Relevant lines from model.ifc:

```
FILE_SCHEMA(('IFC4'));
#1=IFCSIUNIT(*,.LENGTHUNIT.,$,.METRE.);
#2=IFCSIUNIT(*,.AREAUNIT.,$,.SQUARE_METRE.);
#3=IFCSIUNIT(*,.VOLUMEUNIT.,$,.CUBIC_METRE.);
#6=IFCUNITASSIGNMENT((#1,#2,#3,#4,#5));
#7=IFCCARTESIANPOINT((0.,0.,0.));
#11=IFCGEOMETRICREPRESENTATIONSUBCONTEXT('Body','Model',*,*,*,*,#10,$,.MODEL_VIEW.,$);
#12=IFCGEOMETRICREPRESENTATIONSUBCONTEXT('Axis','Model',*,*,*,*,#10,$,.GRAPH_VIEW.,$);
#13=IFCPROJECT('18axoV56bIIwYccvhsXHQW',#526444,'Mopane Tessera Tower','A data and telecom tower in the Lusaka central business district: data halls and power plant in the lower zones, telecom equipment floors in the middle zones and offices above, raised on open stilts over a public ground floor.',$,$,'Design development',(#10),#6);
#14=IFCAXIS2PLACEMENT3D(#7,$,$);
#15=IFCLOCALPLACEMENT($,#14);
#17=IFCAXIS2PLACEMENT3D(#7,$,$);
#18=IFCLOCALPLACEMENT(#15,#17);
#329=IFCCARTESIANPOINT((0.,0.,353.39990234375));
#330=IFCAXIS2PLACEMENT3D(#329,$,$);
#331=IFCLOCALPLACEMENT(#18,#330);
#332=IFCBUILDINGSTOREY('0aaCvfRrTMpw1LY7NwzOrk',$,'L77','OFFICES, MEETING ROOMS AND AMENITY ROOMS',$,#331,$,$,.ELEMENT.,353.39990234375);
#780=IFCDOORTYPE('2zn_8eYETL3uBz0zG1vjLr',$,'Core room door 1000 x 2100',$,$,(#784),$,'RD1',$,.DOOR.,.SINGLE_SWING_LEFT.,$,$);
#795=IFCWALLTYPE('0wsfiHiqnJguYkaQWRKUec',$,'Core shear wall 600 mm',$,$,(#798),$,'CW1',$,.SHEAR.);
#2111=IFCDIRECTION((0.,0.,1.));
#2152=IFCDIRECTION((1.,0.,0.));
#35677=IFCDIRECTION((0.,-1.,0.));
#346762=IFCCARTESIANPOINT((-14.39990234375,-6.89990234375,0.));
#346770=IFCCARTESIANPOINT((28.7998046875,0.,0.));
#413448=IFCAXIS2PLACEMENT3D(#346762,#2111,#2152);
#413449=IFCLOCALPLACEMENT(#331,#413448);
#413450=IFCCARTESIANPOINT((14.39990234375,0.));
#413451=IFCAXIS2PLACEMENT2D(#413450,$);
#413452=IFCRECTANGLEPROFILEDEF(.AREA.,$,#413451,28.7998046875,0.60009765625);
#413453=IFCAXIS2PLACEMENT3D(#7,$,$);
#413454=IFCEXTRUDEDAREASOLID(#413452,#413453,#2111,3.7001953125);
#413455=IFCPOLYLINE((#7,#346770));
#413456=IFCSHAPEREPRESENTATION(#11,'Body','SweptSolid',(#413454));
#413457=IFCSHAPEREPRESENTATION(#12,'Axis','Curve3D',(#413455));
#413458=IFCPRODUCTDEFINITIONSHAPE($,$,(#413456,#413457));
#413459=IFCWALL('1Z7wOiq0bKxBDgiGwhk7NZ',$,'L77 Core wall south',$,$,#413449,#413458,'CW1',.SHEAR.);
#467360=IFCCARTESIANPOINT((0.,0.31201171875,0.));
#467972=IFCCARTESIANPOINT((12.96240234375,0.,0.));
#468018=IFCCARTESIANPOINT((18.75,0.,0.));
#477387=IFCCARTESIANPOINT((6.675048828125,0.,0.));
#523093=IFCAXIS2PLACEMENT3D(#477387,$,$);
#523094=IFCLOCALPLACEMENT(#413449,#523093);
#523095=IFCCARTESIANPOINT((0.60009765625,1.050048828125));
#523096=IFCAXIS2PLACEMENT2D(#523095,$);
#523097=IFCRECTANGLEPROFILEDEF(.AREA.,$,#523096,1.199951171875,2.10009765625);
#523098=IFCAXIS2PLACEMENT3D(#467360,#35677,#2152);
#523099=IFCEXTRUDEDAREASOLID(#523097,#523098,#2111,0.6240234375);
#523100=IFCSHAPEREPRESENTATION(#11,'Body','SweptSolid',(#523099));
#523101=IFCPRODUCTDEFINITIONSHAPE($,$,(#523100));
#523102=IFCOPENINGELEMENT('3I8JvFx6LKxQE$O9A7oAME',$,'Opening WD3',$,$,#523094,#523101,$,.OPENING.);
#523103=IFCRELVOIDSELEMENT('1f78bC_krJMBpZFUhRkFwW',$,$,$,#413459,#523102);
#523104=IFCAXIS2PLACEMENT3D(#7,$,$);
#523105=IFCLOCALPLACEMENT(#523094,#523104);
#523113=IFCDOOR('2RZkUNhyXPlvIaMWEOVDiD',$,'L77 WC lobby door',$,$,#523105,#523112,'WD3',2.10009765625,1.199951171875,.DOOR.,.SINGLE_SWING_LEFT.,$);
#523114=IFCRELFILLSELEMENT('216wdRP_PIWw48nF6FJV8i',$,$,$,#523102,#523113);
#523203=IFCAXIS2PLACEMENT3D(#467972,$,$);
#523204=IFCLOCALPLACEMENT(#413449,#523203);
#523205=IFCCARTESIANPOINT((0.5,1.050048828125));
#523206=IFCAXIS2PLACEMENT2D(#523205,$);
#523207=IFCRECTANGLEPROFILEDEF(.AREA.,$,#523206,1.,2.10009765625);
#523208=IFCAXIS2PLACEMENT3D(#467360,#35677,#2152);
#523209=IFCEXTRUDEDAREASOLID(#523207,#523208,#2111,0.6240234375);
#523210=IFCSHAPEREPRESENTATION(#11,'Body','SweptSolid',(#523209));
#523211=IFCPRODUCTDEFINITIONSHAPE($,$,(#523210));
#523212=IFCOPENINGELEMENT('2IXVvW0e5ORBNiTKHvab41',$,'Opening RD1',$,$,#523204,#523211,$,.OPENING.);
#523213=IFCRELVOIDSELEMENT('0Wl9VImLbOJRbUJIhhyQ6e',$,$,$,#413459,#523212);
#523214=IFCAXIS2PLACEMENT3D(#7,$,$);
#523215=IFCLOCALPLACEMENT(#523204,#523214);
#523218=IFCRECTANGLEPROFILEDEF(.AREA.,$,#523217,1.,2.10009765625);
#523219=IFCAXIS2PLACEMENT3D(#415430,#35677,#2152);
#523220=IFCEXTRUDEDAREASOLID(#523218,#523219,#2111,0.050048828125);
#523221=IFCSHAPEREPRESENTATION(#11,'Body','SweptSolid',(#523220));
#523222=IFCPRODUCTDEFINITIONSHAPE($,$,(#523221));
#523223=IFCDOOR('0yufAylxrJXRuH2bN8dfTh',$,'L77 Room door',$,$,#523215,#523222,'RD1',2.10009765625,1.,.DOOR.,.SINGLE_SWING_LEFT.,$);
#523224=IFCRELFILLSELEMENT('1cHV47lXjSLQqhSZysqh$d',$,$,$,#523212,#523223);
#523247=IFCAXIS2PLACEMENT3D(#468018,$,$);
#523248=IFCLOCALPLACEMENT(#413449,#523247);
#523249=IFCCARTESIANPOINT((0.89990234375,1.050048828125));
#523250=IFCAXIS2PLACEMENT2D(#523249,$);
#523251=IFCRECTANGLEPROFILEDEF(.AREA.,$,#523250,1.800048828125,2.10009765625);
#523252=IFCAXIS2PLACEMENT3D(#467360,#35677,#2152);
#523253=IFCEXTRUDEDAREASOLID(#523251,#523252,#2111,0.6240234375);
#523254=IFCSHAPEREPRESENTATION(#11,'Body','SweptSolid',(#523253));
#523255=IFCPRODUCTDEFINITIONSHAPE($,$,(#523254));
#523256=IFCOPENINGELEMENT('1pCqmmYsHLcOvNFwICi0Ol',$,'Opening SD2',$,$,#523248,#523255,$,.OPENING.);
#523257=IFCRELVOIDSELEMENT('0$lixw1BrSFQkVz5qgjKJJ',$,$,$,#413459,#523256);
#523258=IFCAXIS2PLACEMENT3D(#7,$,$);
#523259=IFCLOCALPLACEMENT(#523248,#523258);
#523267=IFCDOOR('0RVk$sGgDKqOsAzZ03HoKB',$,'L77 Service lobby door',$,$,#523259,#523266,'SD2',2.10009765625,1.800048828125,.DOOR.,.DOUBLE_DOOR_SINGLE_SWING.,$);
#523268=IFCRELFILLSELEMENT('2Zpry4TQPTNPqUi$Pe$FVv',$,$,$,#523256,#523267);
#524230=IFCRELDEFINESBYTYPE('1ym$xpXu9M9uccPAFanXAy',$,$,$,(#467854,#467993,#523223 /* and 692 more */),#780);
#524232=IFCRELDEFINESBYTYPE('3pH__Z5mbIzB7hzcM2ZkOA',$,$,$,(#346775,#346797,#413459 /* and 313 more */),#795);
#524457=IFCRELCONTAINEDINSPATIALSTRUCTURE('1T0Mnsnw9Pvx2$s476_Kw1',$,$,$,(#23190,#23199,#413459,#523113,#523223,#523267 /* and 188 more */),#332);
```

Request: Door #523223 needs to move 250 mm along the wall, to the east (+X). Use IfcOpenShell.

```python
import ifcopenshell
import ifcopenshell.api.geometry
import ifcopenshell.util.placement
import ifcopenshell.util.unit

model = ifcopenshell.open("model.ifc")
unit_scale = ifcopenshell.util.unit.calculate_unit_scale(model)

door = model.by_guid("0yufAylxrJXRuH2bN8dfTh")
opening = door.FillsVoids[0].RelatingOpeningElement
wall = opening.VoidsElements[0].RelatingBuildingElement

wall_matrix = ifcopenshell.util.placement.get_local_placement(wall.ObjectPlacement)
shift = wall_matrix[:3, 0] * 0.25 / unit_scale
before = ifcopenshell.util.placement.get_local_placement(door.ObjectPlacement)[:3, 3].copy()

# The door is placed relative to its opening, so it follows when the opening moves.
matrix = ifcopenshell.util.placement.get_local_placement(opening.ObjectPlacement)
matrix[:3, 3] += shift
ifcopenshell.api.geometry.edit_object_placement(
    model, product=opening, matrix=matrix, is_si=False, should_transform_children=True
)

after = ifcopenshell.util.placement.get_local_placement(door.ObjectPlacement)[:3, 3]
print("door moved by", (after - before).round(3) + 0.0)

model.write("model_v2.ifc")
```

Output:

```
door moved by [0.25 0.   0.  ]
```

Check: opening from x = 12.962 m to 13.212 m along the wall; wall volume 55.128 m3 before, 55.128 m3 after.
